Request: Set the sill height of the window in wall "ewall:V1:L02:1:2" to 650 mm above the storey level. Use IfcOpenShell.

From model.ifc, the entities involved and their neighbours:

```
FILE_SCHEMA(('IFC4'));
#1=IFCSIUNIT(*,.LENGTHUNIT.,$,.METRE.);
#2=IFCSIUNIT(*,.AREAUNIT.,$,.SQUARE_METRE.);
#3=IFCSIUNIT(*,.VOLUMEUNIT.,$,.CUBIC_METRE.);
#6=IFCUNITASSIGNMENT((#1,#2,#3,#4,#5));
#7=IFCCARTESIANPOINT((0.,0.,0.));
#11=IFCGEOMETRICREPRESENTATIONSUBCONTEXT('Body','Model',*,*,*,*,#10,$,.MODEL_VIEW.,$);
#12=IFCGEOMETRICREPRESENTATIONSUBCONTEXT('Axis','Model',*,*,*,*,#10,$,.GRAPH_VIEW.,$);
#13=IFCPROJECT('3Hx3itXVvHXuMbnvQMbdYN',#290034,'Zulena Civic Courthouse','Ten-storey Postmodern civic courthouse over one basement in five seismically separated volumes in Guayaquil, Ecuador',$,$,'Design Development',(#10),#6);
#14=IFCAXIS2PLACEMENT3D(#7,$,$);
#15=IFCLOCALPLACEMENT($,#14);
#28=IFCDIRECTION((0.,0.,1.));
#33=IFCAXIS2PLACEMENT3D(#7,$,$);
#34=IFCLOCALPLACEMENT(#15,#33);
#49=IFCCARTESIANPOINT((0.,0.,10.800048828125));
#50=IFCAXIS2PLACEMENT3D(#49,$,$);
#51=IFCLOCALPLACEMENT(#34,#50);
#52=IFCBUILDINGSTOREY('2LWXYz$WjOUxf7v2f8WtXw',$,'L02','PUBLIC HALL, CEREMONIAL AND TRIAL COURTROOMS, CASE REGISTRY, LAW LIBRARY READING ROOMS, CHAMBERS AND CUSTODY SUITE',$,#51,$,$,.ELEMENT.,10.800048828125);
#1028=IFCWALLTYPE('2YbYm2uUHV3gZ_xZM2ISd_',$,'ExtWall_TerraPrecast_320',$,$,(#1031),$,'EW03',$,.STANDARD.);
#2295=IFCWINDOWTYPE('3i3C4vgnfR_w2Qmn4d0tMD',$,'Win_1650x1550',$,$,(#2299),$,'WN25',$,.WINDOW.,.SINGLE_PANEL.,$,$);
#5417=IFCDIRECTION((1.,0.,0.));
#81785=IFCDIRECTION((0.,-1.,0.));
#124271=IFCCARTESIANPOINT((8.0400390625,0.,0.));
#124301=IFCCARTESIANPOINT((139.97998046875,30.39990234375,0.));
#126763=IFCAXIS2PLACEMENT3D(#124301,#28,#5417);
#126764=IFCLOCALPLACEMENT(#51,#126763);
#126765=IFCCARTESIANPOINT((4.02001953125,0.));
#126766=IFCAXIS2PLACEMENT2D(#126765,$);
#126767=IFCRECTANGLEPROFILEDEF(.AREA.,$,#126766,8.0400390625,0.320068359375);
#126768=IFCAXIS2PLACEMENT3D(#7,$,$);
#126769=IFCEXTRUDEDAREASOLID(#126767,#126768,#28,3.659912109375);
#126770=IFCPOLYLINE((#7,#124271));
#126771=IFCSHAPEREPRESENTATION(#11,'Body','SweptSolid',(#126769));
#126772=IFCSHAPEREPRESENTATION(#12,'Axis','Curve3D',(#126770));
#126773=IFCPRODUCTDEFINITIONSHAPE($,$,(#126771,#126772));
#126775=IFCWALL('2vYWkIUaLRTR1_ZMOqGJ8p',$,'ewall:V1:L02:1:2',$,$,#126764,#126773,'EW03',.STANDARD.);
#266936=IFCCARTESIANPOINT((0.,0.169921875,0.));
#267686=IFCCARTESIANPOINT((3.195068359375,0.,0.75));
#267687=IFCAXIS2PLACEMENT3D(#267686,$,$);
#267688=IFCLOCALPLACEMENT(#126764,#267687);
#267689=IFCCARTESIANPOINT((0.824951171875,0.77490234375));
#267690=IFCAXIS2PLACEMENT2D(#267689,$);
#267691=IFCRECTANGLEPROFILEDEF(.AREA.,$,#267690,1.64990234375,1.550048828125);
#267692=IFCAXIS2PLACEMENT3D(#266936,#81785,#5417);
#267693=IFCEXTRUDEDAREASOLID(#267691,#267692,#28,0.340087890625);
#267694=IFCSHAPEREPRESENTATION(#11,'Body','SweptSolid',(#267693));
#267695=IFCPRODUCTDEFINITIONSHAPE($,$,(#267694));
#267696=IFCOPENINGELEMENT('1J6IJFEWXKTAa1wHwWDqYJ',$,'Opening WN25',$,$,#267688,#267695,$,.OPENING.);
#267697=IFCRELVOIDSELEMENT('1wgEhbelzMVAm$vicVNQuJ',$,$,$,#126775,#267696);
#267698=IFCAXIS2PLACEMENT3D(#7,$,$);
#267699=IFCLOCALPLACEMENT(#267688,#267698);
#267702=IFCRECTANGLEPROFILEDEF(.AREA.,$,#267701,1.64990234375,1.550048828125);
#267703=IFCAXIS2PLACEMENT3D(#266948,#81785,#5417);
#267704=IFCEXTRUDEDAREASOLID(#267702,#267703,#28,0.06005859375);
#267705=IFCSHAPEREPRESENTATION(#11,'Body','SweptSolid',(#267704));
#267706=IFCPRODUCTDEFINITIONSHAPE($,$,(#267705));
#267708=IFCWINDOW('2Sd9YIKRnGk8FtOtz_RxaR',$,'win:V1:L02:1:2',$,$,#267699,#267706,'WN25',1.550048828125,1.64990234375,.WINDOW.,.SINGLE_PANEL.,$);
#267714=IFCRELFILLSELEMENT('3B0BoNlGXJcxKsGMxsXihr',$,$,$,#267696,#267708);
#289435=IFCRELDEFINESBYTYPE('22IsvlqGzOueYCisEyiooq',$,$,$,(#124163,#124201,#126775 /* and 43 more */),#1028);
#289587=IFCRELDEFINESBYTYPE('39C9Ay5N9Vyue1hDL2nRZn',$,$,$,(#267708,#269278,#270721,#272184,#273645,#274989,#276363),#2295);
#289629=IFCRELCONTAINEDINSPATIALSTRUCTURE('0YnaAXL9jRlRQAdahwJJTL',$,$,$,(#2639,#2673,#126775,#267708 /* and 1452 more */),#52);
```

```python
import numpy as np
import ifcopenshell
import ifcopenshell.api.geometry
import ifcopenshell.geom
import ifcopenshell.util.element
import ifcopenshell.util.placement
import ifcopenshell.util.shape
import ifcopenshell.util.unit

model = ifcopenshell.open("model.ifc")
unit_scale = ifcopenshell.util.unit.calculate_unit_scale(model)

window = model.by_guid("2Sd9YIKRnGk8FtOtz_RxaR")
opening = window.FillsVoids[0].RelatingOpeningElement
storey = ifcopenshell.util.element.get_container(window, ifc_class="IfcBuildingStorey")
level = ifcopenshell.util.placement.get_local_placement(storey.ObjectPlacement)[2, 3]

# The opening's origin need not be at the sill, so measure its lowest point.
shape = ifcopenshell.geom.create_shape(ifcopenshell.geom.settings(), opening)
bottom = ifcopenshell.util.shape.get_shape_bottom_elevation(shape, shape.geometry) / unit_scale
dz = level + 0.65 - bottom

shift = np.array([0.0, 0.0, dz])
# The window is placed relative to its opening, so it follows when the opening moves.
matrix = ifcopenshell.util.placement.get_local_placement(opening.ObjectPlacement)
matrix[:3, 3] += shift
ifcopenshell.api.geometry.edit_object_placement(
    model, product=opening, matrix=matrix, is_si=False, should_transform_children=True
)

print(f"moved by {dz * unit_scale:+.3f} m")

model.write("model_updated.ifc")
```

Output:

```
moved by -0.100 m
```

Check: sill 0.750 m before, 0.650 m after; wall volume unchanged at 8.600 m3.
